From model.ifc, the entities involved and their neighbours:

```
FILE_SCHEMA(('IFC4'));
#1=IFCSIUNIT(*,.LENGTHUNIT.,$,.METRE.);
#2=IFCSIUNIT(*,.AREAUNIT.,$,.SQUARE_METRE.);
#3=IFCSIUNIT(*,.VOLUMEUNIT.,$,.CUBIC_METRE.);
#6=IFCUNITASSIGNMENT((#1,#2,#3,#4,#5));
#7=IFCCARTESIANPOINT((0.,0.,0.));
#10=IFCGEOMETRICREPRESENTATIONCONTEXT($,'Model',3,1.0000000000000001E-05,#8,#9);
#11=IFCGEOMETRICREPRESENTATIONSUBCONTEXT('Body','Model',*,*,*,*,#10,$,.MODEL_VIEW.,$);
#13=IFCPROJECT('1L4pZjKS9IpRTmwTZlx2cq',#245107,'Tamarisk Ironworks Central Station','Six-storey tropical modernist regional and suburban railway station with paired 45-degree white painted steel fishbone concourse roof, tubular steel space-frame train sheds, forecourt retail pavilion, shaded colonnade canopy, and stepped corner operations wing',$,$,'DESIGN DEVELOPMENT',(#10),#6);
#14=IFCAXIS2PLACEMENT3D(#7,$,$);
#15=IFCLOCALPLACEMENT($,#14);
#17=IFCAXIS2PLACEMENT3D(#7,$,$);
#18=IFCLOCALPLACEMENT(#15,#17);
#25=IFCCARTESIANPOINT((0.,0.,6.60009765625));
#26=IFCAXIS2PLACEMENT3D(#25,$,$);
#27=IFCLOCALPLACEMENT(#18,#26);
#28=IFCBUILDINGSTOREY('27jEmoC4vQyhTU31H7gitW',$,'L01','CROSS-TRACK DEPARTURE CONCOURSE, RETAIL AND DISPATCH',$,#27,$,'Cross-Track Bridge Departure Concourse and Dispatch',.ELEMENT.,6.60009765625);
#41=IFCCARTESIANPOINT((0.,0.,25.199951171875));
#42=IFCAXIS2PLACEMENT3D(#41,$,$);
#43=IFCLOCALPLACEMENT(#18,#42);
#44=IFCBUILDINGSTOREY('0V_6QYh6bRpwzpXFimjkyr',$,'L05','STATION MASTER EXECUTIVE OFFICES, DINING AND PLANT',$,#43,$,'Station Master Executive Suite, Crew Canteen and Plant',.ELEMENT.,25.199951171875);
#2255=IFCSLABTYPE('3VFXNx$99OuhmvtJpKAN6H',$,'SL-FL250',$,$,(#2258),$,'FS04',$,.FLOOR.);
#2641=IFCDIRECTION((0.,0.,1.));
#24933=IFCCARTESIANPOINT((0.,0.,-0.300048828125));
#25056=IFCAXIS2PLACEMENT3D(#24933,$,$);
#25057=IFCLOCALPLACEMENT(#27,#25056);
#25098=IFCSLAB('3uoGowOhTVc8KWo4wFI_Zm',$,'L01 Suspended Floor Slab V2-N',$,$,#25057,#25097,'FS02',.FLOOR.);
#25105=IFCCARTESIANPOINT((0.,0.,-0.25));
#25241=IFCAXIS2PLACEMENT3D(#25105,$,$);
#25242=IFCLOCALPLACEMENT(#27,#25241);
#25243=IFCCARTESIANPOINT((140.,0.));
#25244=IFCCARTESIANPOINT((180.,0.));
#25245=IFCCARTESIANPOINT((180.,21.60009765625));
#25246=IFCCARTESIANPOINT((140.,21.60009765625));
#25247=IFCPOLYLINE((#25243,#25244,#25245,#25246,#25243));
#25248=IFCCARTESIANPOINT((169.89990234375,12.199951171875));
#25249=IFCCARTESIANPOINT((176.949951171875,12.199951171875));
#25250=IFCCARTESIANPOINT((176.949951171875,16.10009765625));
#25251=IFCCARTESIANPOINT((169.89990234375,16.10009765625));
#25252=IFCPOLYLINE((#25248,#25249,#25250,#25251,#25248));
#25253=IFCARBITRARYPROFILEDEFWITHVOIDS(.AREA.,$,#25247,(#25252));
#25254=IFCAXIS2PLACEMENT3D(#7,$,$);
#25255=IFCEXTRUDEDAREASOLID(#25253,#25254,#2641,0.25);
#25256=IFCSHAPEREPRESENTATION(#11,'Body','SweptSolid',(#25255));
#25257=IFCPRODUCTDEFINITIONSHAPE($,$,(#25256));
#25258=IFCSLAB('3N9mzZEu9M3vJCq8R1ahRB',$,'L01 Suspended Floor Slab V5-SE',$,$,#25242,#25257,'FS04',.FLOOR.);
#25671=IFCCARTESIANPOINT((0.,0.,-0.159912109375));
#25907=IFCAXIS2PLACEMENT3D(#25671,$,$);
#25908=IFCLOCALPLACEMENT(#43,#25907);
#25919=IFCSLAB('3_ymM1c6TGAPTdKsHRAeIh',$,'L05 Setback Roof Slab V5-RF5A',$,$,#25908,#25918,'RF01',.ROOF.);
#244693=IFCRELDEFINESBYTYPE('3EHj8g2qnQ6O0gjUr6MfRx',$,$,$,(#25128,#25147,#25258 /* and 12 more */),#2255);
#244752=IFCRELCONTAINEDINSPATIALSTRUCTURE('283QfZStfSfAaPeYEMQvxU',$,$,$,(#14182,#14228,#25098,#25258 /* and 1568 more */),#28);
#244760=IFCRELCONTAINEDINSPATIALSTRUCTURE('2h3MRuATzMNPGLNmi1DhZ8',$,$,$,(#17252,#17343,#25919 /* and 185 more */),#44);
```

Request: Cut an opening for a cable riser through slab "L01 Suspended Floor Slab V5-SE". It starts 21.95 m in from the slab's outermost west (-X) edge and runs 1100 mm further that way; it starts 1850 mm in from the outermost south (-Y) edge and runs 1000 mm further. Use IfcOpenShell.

```python
import numpy as np
import ifcopenshell
import ifcopenshell.api.feature
import ifcopenshell.api.geometry
import ifcopenshell.api.root
import ifcopenshell.geom
import ifcopenshell.util.placement
import ifcopenshell.util.representation
import ifcopenshell.util.shape
import ifcopenshell.util.unit

model = ifcopenshell.open("model.ifc")
unit_scale = ifcopenshell.util.unit.calculate_unit_scale(model)
settings = ifcopenshell.geom.settings()


def volume(element):
    """Net volume in cubic metres, openings subtracted."""
    shape = ifcopenshell.geom.create_shape(settings, element)
    return ifcopenshell.util.shape.get_volume(shape.geometry)


slab = model.by_guid("3N9mzZEu9M3vJCq8R1ahRB")
before = volume(slab)

# Extent in the slab's own axes, in metres. The edges named are its -X and -Y sides.
slab_shape = ifcopenshell.geom.create_shape(settings, slab)
vertices = ifcopenshell.util.shape.get_vertices(slab_shape.geometry)
x_min, y_min, bottom = vertices.min(axis=0)
top = vertices[:, 2].max()

opening = ifcopenshell.api.root.create_entity(model, ifc_class="IfcOpeningElement", name="Cable riser opening", predefined_type="OPENING")
context = ifcopenshell.util.representation.get_context(model, "Model", "Body", "MODEL_VIEW")
width, depth = 1.1, 1
outline = [(0.0, 0.0), (width, 0.0), (width, depth), (0.0, depth), (0.0, 0.0)]
# Overshoot both faces by 50 mm so the cut is clean.
shape = ifcopenshell.api.geometry.add_slab_representation(
    model, context=context, depth=top - bottom + 0.1, polyline=outline
)
ifcopenshell.api.geometry.assign_representation(model, product=opening, representation=shape)

matrix = ifcopenshell.util.placement.get_local_placement(slab.ObjectPlacement)
matrix[:, 3] = matrix @ np.append(np.array([x_min + 21.95, y_min + 1.85, bottom - 0.05]) / unit_scale, 1.0)
ifcopenshell.api.geometry.edit_object_placement(model, product=opening, matrix=matrix, is_si=False)
ifcopenshell.api.feature.add_feature(model, feature=opening, element=slab)

after = volume(slab)

print(f"slab volume {before:.3f} -> {after:.3f} m3")

model.write("model_rev.ifc")
```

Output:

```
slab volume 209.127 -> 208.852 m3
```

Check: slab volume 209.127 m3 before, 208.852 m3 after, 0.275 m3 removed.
